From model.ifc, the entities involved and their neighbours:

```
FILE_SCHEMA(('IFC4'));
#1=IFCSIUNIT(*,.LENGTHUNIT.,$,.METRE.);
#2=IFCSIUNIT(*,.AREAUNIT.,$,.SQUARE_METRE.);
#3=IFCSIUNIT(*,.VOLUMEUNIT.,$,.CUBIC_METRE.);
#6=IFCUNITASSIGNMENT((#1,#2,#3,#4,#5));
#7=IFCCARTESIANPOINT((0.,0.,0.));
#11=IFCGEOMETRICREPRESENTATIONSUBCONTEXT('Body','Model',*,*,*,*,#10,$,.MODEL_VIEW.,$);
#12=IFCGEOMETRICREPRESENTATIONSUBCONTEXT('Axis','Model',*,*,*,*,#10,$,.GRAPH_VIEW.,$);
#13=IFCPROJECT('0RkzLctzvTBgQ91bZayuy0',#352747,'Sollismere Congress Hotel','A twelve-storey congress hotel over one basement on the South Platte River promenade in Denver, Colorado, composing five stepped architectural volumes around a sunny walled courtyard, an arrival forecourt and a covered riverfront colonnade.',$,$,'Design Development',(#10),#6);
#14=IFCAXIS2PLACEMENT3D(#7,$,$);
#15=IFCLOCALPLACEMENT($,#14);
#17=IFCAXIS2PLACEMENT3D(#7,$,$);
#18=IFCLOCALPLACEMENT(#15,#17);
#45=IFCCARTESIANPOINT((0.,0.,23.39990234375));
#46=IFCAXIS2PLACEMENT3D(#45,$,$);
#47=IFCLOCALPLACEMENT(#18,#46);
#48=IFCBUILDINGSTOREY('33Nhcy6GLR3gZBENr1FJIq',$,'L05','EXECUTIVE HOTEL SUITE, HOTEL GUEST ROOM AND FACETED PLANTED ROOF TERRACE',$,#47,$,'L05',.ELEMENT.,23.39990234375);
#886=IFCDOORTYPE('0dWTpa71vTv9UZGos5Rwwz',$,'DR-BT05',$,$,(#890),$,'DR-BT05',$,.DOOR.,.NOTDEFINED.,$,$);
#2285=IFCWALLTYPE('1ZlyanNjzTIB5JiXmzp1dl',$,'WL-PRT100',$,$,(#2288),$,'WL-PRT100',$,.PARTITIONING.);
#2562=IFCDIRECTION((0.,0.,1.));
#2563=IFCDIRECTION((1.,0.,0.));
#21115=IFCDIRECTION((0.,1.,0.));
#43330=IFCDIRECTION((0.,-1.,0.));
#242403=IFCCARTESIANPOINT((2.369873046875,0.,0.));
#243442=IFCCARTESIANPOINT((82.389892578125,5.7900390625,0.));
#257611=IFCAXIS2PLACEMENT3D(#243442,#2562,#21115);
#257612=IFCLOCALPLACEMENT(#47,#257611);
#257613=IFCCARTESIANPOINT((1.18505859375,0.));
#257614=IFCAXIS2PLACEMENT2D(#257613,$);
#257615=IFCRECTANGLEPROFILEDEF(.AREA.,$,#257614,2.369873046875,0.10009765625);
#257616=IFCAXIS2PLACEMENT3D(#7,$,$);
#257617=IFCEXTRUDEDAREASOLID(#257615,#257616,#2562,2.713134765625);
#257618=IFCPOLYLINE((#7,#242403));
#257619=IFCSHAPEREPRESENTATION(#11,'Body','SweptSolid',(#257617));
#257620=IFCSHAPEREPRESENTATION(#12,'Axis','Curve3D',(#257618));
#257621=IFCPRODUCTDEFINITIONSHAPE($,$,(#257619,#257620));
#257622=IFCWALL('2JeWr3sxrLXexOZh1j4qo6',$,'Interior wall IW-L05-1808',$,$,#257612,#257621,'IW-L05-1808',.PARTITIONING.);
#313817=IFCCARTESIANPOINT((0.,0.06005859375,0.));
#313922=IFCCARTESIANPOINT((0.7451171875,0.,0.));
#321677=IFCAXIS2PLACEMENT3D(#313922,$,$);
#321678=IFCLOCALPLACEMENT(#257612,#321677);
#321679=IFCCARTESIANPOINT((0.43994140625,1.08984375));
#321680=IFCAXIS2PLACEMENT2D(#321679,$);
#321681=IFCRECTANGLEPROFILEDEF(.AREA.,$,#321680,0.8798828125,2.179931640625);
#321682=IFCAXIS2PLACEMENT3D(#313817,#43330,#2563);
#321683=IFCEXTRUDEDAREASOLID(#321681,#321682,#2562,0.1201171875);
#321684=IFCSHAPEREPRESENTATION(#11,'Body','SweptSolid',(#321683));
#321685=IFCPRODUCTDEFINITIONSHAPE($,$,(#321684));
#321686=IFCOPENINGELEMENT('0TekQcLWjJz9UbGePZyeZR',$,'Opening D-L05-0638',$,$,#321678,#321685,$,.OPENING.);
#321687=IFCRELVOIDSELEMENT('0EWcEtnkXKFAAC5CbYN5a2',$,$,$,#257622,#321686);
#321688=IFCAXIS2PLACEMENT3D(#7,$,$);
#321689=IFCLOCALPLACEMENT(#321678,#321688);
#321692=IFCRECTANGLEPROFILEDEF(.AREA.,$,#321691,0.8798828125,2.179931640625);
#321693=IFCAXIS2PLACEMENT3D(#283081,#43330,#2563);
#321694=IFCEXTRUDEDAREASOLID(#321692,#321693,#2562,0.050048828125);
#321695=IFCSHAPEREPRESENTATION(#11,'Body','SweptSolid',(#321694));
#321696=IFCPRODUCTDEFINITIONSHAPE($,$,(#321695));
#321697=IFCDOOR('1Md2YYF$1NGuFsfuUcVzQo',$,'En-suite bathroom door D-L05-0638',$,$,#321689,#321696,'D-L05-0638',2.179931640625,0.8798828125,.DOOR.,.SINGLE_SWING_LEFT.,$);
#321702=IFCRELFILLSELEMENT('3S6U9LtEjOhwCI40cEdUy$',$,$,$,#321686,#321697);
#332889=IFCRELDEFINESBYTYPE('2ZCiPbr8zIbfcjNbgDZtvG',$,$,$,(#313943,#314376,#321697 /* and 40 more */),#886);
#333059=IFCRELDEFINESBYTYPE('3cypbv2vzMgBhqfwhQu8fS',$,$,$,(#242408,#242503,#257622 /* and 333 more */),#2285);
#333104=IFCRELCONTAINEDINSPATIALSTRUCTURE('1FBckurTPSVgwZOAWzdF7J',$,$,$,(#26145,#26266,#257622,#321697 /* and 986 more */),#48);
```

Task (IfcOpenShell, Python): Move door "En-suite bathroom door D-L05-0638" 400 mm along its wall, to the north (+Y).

```python
import ifcopenshell
import ifcopenshell.api.geometry
import ifcopenshell.util.placement
import ifcopenshell.util.unit

model = ifcopenshell.open("model.ifc")
unit_scale = ifcopenshell.util.unit.calculate_unit_scale(model)

door = model.by_guid("1Md2YYF$1NGuFsfuUcVzQo")
opening = door.FillsVoids[0].RelatingOpeningElement
wall = opening.VoidsElements[0].RelatingBuildingElement

wall_matrix = ifcopenshell.util.placement.get_local_placement(wall.ObjectPlacement)
shift = wall_matrix[:3, 0] * 0.4 / unit_scale
before = ifcopenshell.util.placement.get_local_placement(door.ObjectPlacement)[:3, 3].copy()

# The door is placed relative to its opening, so it follows when the opening moves.
matrix = ifcopenshell.util.placement.get_local_placement(opening.ObjectPlacement)
matrix[:3, 3] += shift
ifcopenshell.api.geometry.edit_object_placement(
    model, product=opening, matrix=matrix, is_si=False, should_transform_children=True
)

after = ifcopenshell.util.placement.get_local_placement(door.ObjectPlacement)[:3, 3]
print("door moved by", (after - before).round(3) + 0.0)

model.write("model-out.ifc")
```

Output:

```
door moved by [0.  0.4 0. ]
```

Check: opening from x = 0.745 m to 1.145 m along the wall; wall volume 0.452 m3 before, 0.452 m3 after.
